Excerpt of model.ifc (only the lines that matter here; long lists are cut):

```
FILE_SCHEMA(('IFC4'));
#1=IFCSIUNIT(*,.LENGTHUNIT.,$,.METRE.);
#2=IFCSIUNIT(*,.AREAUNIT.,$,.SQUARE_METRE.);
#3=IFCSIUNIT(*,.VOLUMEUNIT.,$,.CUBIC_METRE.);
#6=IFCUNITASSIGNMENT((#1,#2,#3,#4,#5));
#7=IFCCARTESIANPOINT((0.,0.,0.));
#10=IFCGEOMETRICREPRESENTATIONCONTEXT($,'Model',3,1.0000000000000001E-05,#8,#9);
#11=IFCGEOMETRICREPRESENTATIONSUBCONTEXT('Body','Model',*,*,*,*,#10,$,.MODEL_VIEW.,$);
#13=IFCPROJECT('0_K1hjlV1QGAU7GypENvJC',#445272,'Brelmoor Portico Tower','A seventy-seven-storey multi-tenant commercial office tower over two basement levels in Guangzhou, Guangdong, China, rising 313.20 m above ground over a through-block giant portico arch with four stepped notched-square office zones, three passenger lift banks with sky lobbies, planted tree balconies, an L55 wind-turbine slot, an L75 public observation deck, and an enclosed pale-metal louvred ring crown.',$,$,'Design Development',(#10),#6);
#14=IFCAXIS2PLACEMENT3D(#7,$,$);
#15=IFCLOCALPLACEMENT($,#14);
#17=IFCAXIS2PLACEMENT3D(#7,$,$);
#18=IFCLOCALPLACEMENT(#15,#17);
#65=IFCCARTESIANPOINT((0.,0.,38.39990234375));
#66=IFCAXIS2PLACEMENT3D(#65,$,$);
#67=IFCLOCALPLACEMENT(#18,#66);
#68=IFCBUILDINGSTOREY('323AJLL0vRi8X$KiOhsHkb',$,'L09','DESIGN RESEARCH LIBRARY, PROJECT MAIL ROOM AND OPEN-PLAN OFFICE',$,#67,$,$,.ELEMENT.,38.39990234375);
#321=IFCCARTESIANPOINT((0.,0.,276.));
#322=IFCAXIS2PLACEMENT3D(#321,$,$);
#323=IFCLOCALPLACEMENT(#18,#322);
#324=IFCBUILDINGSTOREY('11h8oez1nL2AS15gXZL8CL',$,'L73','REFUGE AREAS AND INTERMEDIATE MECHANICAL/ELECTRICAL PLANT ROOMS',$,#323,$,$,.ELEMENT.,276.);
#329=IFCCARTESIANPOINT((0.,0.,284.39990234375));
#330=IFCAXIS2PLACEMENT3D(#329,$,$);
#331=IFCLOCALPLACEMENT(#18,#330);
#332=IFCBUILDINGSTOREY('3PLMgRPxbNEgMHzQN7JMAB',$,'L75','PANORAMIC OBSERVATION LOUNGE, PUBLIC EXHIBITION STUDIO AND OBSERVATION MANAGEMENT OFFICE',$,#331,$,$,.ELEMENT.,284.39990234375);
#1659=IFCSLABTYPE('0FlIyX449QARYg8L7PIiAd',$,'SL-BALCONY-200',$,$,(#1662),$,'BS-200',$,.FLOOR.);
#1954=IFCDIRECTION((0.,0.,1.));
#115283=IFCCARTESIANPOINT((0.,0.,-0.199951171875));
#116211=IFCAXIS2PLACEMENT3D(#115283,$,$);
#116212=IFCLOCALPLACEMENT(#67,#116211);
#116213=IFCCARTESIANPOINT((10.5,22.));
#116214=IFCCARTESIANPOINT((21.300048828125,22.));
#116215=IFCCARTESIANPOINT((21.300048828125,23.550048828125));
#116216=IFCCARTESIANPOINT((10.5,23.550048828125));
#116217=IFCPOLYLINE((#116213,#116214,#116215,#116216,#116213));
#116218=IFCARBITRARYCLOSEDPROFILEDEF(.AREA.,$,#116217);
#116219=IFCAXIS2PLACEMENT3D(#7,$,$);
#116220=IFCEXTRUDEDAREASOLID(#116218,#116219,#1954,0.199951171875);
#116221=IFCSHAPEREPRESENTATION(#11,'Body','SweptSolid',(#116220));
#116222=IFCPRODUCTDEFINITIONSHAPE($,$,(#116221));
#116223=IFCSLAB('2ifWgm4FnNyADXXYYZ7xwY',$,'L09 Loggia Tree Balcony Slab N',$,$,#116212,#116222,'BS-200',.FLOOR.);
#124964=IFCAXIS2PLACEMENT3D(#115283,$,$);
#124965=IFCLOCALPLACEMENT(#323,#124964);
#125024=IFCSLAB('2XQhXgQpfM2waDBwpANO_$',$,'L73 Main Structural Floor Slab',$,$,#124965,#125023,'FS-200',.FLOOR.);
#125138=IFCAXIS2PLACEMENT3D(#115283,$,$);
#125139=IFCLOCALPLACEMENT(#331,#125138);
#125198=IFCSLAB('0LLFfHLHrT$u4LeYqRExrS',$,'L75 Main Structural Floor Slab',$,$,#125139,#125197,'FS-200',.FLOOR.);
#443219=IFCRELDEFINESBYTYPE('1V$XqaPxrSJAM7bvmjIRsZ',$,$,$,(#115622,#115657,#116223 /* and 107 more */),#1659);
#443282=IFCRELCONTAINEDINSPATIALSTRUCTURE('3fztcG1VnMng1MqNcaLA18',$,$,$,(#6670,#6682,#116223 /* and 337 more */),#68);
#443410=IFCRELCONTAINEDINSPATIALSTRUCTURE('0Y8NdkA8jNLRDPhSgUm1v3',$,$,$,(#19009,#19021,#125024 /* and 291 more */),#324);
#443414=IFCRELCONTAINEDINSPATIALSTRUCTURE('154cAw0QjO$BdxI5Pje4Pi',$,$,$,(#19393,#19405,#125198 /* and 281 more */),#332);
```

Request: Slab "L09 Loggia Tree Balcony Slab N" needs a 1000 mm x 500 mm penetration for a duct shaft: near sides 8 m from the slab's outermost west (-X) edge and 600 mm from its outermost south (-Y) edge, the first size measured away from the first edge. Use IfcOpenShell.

```python
import numpy as np
import ifcopenshell
import ifcopenshell.api.feature
import ifcopenshell.api.geometry
import ifcopenshell.api.root
import ifcopenshell.geom
import ifcopenshell.util.placement
import ifcopenshell.util.representation
import ifcopenshell.util.shape
import ifcopenshell.util.unit

model = ifcopenshell.open("model.ifc")
unit_scale = ifcopenshell.util.unit.calculate_unit_scale(model)
settings = ifcopenshell.geom.settings()


def volume(element):
    """Net volume in cubic metres, openings subtracted."""
    shape = ifcopenshell.geom.create_shape(settings, element)
    return ifcopenshell.util.shape.get_volume(shape.geometry)


slab = model.by_guid("2ifWgm4FnNyADXXYYZ7xwY")
before = volume(slab)

# Extent in the slab's own axes, in metres. The edges named are its -X and -Y sides.
slab_shape = ifcopenshell.geom.create_shape(settings, slab)
vertices = ifcopenshell.util.shape.get_vertices(slab_shape.geometry)
x_min, y_min, bottom = vertices.min(axis=0)
top = vertices[:, 2].max()

opening = ifcopenshell.api.root.create_entity(model, ifc_class="IfcOpeningElement", name="Duct shaft opening", predefined_type="OPENING")
context = ifcopenshell.util.representation.get_context(model, "Model", "Body", "MODEL_VIEW")
width, depth = 1, 0.5
outline = [(0.0, 0.0), (width, 0.0), (width, depth), (0.0, depth), (0.0, 0.0)]
# Overshoot both faces by 50 mm so the cut is clean.
shape = ifcopenshell.api.geometry.add_slab_representation(
    model, context=context, depth=top - bottom + 0.1, polyline=outline
)
ifcopenshell.api.geometry.assign_representation(model, product=opening, representation=shape)

matrix = ifcopenshell.util.placement.get_local_placement(slab.ObjectPlacement)
matrix[:, 3] = matrix @ np.append(np.array([x_min + 8, y_min + 0.6, bottom - 0.05]) / unit_scale, 1.0)
ifcopenshell.api.geometry.edit_object_placement(model, product=opening, matrix=matrix, is_si=False)
ifcopenshell.api.feature.add_feature(model, feature=opening, element=slab)

after = volume(slab)

print(f"slab volume {before:.3f} -> {after:.3f} m3")

model.write("model_v2.ifc")
```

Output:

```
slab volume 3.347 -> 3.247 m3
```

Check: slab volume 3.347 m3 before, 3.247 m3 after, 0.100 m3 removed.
